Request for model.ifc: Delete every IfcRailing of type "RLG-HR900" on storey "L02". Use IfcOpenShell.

First a look at what the model holds.

```python
import ifcopenshell
import ifcopenshell.util.element

model = ifcopenshell.open("model.ifc")
print(model.schema)
storey = next(s for s in model.by_type("IfcBuildingStorey") if s.Name == "L02")
railings = [e for e in ifcopenshell.util.element.get_decomposition(storey) if e.is_a("IfcRailing")]
seen = {}
for e in railings:
    element_type = ifcopenshell.util.element.get_type(e)
    name = element_type.Name if element_type not in (None, e) else None
    seen[name] = seen.get(name, 0) + 1
for name, count in sorted(seen.items(), key=str):
    print(count, "x", name)
```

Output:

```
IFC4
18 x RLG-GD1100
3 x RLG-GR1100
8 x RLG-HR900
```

```python
import ifcopenshell
import ifcopenshell.api.root
import ifcopenshell.util.element

model = ifcopenshell.open("model.ifc")

storey = next(s for s in model.by_type("IfcBuildingStorey") if s.Name == "L02")
railings = [e for e in ifcopenshell.util.element.get_decomposition(storey) if e.is_a("IfcRailing")]
targets = [e for e in railings if (t := ifcopenshell.util.element.get_type(e)) not in (None, e) and t.Name == "RLG-HR900"]

for e in targets:
    ifcopenshell.api.root.remove_product(model, product=e)
print(len(targets), "removed")

model.write("model_updated.ifc")
```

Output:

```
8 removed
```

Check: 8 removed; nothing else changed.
